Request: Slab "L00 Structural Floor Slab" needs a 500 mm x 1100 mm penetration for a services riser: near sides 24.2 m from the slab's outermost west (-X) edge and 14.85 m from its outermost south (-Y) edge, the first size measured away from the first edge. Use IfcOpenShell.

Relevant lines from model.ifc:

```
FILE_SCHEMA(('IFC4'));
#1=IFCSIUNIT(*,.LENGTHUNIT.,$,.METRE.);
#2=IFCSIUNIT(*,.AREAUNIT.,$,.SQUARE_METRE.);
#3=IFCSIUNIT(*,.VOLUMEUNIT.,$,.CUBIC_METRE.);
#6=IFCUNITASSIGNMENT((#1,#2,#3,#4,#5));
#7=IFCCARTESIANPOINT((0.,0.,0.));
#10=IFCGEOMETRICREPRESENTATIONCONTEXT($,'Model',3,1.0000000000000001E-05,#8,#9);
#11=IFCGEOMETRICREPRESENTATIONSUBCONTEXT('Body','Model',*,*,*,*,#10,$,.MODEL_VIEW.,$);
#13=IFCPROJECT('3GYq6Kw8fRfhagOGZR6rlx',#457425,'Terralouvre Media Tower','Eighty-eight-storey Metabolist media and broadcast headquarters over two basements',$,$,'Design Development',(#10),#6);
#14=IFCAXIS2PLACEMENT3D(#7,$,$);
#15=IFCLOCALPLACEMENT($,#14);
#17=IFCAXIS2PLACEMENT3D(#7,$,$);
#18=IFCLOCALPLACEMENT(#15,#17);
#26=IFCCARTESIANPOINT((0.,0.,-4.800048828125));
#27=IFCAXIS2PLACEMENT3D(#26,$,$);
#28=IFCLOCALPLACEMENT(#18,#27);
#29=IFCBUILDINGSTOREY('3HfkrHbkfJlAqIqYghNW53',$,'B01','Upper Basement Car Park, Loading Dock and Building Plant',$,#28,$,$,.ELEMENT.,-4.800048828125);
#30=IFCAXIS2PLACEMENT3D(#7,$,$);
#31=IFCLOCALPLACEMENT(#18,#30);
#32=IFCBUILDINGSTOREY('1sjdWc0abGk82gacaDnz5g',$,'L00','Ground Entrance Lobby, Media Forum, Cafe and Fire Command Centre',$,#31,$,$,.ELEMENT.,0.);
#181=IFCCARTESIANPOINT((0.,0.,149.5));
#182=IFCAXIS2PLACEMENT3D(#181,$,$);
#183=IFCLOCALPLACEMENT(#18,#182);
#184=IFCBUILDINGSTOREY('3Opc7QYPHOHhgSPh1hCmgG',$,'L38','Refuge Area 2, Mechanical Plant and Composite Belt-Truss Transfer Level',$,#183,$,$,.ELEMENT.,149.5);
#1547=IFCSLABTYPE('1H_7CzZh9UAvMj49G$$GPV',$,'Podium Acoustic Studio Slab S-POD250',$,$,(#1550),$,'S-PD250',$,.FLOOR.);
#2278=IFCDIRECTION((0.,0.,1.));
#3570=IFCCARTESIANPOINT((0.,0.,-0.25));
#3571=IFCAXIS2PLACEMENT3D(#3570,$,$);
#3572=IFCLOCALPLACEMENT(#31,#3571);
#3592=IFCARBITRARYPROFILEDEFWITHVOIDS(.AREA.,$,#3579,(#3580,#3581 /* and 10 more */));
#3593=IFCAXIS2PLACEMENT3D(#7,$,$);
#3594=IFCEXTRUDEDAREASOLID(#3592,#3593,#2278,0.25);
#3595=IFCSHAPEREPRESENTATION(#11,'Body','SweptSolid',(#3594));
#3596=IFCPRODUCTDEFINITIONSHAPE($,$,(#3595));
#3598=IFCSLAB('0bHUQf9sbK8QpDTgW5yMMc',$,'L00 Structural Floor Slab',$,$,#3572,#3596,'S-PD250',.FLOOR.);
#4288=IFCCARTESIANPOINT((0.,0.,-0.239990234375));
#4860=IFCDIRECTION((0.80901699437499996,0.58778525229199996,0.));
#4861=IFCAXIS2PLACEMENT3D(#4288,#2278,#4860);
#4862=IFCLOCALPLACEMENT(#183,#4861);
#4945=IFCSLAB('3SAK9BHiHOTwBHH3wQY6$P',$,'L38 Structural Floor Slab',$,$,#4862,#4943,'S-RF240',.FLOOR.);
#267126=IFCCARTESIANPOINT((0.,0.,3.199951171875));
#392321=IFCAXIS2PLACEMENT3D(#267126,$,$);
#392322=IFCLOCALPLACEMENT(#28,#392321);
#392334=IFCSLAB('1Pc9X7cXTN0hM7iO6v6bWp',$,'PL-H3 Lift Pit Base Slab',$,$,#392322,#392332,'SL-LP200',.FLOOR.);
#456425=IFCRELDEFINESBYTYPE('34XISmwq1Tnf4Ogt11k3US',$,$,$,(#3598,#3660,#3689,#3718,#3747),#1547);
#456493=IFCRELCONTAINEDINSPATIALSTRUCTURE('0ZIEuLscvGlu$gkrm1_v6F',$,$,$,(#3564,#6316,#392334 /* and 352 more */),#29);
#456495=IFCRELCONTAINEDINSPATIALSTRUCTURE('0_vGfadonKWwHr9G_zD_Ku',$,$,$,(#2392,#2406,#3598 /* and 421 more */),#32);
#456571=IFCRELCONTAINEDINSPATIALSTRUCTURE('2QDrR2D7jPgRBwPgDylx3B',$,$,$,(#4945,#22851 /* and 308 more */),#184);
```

```python
import numpy as np
import ifcopenshell
import ifcopenshell.api.feature
import ifcopenshell.api.geometry
import ifcopenshell.api.root
import ifcopenshell.geom
import ifcopenshell.util.placement
import ifcopenshell.util.representation
import ifcopenshell.util.shape
import ifcopenshell.util.unit

model = ifcopenshell.open("model.ifc")
unit_scale = ifcopenshell.util.unit.calculate_unit_scale(model)
settings = ifcopenshell.geom.settings()


def volume(element):
    """Net volume in cubic metres, openings subtracted."""
    shape = ifcopenshell.geom.create_shape(settings, element)
    return ifcopenshell.util.shape.get_volume(shape.geometry)


slab = model.by_guid("0bHUQf9sbK8QpDTgW5yMMc")
before = volume(slab)

# Extent in the slab's own axes, in metres. The edges named are its -X and -Y sides.
slab_shape = ifcopenshell.geom.create_shape(settings, slab)
vertices = ifcopenshell.util.shape.get_vertices(slab_shape.geometry)
x_min, y_min, bottom = vertices.min(axis=0)
top = vertices[:, 2].max()

opening = ifcopenshell.api.root.create_entity(model, ifc_class="IfcOpeningElement", name="Services riser opening", predefined_type="OPENING")
context = ifcopenshell.util.representation.get_context(model, "Model", "Body", "MODEL_VIEW")
width, depth = 0.5, 1.1
outline = [(0.0, 0.0), (width, 0.0), (width, depth), (0.0, depth), (0.0, 0.0)]
# Overshoot both faces by 50 mm so the cut is clean.
shape = ifcopenshell.api.geometry.add_slab_representation(
    model, context=context, depth=top - bottom + 0.1, polyline=outline
)
ifcopenshell.api.geometry.assign_representation(model, product=opening, representation=shape)

matrix = ifcopenshell.util.placement.get_local_placement(slab.ObjectPlacement)
matrix[:, 3] = matrix @ np.append(np.array([x_min + 24.2, y_min + 14.85, bottom - 0.05]) / unit_scale, 1.0)
ifcopenshell.api.geometry.edit_object_placement(model, product=opening, matrix=matrix, is_si=False)
ifcopenshell.api.feature.add_feature(model, feature=opening, element=slab)

after = volume(slab)

print(f"slab volume {before:.3f} -> {after:.3f} m3")

model.write("model_edited.ifc")
```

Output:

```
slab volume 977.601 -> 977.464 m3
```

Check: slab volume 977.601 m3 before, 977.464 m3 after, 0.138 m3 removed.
